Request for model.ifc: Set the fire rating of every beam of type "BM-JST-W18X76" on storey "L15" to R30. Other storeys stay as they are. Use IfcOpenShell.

First a look at what the model holds.

```python
import ifcopenshell
import ifcopenshell.util.element

model = ifcopenshell.open("model.ifc")
print(model.schema)
storey = next(s for s in model.by_type("IfcBuildingStorey") if s.Name == "L15")
beams = [e for e in ifcopenshell.util.element.get_decomposition(storey) if e.is_a("IfcBeam")]
seen = {}
for e in beams:
    element_type = ifcopenshell.util.element.get_type(e)
    key = (element_type.Name if element_type != e and element_type else None, ifcopenshell.util.element.get_pset(e, "Pset_BeamCommon", "FireRating"))
    seen[key] = seen.get(key, 0) + 1
for (name, value), count in sorted(seen.items(), key=str):
    print(count, "x", name, "|", value)
```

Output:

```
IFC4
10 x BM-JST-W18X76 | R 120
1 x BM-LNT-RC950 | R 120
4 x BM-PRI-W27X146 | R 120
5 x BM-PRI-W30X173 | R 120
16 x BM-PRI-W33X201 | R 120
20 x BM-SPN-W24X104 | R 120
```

```python
import ifcopenshell
import ifcopenshell.api.pset
import ifcopenshell.util.element

model = ifcopenshell.open("model.ifc")

storey = next(s for s in model.by_type("IfcBuildingStorey") if s.Name == "L15")
beams = [e for e in ifcopenshell.util.element.get_decomposition(storey) if e.is_a("IfcBeam")]

count = 0
for e in beams:
    element_type = ifcopenshell.util.element.get_type(e)
    if element_type in (None, e) or element_type.Name != "BM-JST-W18X76":
        continue
    found = ifcopenshell.util.element.get_pset(e, "Pset_BeamCommon", should_inherit=False)
    if found:
        pset = model.by_id(found["id"])
        if len(ifcopenshell.util.element.get_elements_by_pset(pset)) > 1:
            pset = ifcopenshell.api.pset.unshare_pset(model, products=[e], pset=pset)[0]
    else:
        pset = ifcopenshell.api.pset.add_pset(model, product=e, name="Pset_BeamCommon")
    ifcopenshell.api.pset.edit_pset(model, pset=pset, properties={"FireRating": "R30"})
    count += 1

print(count, "beams updated")

model.write("model_rev.ifc")
```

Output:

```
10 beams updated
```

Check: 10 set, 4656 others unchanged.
